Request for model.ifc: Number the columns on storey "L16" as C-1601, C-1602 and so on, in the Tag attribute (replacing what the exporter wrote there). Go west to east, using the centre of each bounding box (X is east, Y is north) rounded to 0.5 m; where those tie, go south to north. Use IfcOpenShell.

First a look at what the model holds.

```python
import ifcopenshell
import ifcopenshell.util.element
import ifcopenshell.util.placement

model = ifcopenshell.open("model.ifc")
print(model.schema)
storey = next(s for s in model.by_type("IfcBuildingStorey") if s.Name == "L16")
columns = [e for e in ifcopenshell.util.element.get_decomposition(storey) if e.is_a("IfcColumn")]
for e in sorted(columns, key=lambda e: e.id()):
    origin = ifcopenshell.util.placement.get_local_placement(e.ObjectPlacement)[:3, 3]
    print(e.id(), e.Tag, e.Name, origin.round(2) + 0.0, sep=" | ")
```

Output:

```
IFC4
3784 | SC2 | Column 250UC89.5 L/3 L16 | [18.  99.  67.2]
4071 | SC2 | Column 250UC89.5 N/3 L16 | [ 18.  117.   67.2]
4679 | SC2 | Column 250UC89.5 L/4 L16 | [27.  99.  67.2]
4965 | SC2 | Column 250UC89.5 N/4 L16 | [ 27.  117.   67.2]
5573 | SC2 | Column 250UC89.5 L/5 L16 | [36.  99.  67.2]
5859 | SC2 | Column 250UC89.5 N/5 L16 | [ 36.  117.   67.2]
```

```python
import ifcopenshell
import ifcopenshell.geom
import ifcopenshell.util.element
import ifcopenshell.util.shape

model = ifcopenshell.open("model.ifc")
settings = ifcopenshell.geom.settings()
settings.set("use-world-coords", True)


def centre(element):
    shape = ifcopenshell.geom.create_shape(settings, element)
    return ifcopenshell.util.shape.get_bbox_centroid(shape.geometry)


storey = next(s for s in model.by_type("IfcBuildingStorey") if s.Name == "L16")
columns = [e for e in ifcopenshell.util.element.get_decomposition(storey) if e.is_a("IfcColumn")]

# Insertion points can sit at a corner or the storey origin, so sort by the geometry (in metres).
centres = {e: centre(e) for e in columns}
columns.sort(key=lambda e: (round(centres[e][0] / 0.5), centres[e][1]))

for i, e in enumerate(columns, start=1):
    number = f"C-16{i:02d}"
    e.Tag = number
    print(e.id(), number)

model.write("model_updated.ifc")
```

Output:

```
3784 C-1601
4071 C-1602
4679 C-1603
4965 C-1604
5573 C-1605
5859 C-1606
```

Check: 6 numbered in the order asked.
